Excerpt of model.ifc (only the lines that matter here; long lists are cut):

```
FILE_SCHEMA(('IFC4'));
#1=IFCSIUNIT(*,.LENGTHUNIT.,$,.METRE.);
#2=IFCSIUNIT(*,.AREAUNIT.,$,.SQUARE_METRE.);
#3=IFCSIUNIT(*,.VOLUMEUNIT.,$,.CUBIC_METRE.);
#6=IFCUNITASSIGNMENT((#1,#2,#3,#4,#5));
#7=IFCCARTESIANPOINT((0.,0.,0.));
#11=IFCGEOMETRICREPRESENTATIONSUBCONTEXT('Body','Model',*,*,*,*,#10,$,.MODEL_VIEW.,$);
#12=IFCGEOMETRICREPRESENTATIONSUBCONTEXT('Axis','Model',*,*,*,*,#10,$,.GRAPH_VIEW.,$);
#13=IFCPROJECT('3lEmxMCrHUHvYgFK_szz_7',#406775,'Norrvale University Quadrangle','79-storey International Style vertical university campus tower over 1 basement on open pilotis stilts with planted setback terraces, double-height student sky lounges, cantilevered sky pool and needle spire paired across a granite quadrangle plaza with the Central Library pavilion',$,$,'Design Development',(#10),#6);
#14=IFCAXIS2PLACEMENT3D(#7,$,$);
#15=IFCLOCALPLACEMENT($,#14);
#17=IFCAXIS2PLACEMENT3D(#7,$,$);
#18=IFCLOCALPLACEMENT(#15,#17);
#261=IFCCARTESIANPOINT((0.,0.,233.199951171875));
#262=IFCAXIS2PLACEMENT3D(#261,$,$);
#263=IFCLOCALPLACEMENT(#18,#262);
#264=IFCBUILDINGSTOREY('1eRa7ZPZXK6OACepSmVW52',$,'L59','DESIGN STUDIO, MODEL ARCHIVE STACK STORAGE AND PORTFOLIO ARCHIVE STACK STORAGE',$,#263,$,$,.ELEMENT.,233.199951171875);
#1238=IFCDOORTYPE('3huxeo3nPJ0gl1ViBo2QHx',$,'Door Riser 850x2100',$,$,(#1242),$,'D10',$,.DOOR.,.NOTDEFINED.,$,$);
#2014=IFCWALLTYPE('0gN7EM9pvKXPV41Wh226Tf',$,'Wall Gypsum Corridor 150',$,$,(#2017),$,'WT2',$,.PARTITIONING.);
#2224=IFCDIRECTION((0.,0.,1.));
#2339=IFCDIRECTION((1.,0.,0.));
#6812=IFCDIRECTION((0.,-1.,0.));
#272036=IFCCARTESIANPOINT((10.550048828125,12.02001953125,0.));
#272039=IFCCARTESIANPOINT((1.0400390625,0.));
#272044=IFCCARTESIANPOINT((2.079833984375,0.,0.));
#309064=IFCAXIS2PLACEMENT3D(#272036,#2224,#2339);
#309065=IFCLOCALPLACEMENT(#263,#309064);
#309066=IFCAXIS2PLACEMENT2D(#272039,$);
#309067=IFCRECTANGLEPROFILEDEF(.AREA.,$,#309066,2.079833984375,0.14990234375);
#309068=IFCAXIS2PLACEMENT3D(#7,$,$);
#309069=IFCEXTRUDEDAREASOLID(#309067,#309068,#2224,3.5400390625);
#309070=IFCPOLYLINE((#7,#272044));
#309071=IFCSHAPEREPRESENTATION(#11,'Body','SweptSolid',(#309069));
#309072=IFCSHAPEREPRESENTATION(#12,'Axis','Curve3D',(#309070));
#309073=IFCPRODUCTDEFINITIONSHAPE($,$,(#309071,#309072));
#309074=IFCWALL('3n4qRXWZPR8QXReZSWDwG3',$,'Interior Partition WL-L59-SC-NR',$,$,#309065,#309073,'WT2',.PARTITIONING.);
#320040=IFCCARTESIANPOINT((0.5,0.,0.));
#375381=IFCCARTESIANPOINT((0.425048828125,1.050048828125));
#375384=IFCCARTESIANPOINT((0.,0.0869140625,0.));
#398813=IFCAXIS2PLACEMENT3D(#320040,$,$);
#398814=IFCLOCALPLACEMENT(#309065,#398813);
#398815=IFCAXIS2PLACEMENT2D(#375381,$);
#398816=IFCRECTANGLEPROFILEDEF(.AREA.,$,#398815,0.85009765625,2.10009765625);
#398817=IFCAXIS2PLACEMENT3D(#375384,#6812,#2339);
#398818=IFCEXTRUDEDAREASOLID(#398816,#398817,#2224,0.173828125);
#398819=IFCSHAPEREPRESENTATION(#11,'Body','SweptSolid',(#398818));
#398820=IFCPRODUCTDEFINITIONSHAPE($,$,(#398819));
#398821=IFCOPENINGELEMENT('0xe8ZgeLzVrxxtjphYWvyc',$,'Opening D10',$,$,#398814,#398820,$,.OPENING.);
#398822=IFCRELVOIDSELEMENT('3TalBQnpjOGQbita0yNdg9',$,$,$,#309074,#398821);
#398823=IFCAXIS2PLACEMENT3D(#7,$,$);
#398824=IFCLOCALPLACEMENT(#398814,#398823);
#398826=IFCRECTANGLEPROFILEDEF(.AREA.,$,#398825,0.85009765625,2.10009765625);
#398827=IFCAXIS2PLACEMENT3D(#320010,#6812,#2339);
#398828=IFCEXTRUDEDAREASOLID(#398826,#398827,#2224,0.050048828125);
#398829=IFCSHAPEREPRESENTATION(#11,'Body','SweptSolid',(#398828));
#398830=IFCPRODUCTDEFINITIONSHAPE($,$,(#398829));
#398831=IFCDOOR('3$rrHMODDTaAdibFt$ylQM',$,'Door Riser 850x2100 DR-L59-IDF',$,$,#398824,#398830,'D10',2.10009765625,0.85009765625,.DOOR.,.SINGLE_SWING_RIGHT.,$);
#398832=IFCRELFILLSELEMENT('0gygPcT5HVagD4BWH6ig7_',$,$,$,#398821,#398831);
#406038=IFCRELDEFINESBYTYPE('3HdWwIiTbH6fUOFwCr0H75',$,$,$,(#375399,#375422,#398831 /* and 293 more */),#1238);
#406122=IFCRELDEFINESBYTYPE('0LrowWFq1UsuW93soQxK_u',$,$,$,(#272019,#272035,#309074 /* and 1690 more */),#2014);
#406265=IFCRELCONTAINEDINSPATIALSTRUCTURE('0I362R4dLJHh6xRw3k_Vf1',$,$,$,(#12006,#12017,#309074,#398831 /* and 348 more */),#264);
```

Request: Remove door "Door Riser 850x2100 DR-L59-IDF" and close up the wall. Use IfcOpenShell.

```python
import ifcopenshell
import ifcopenshell.api.feature
import ifcopenshell.api.root
import ifcopenshell.geom
import ifcopenshell.util.shape

model = ifcopenshell.open("model.ifc")
settings = ifcopenshell.geom.settings()


def volume(element):
    """Net volume in cubic metres, openings subtracted."""
    shape = ifcopenshell.geom.create_shape(settings, element)
    return ifcopenshell.util.shape.get_volume(shape.geometry)


door = model.by_guid("3$rrHMODDTaAdibFt$ylQM")
opening = door.FillsVoids[0].RelatingOpeningElement
wall = opening.VoidsElements[0].RelatingBuildingElement
before = volume(wall)

ifcopenshell.api.root.remove_product(model, product=door)
ifcopenshell.api.feature.remove_feature(model, feature=opening)

after = volume(wall)

print(f"wall volume {before:.3f} -> {after:.3f} m3")

model.write("model_edited.ifc")
```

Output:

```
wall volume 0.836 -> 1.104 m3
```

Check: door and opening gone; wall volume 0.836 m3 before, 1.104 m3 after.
